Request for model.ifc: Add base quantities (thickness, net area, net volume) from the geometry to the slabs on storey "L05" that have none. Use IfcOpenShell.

First a look at what the model holds.

```python
import ifcopenshell
import ifcopenshell.util.element
import ifcopenshell.util.unit

model = ifcopenshell.open("model.ifc")
print(model.schema)
for unit_type in ("LENGTHUNIT", "AREAUNIT", "VOLUMEUNIT"):
    print(unit_type, ifcopenshell.util.unit.calculate_unit_scale(model, unit_type))
storey = next(s for s in model.by_type("IfcBuildingStorey") if s.Name == "L05")
slabs = [e for e in ifcopenshell.util.element.get_decomposition(storey) if e.is_a("IfcSlab")]
for e in sorted(slabs, key=lambda e: e.id()):
    print(e.id(), e.is_a(), e.Name, list(ifcopenshell.util.element.get_psets(e, qtos_only=True)), sep=" | ")
```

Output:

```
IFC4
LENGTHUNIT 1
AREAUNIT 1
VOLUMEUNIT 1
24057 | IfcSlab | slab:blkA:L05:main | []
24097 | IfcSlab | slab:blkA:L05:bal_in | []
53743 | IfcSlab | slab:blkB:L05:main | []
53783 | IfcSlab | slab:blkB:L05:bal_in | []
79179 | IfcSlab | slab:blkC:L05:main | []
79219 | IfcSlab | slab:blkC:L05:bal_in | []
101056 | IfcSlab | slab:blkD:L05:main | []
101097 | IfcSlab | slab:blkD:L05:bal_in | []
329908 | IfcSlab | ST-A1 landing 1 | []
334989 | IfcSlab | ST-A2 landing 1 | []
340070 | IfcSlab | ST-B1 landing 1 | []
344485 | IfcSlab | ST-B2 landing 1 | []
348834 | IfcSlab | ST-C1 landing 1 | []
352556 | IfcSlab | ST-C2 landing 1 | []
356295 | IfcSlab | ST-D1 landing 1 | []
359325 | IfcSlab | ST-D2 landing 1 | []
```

```python
import ifcopenshell
import ifcopenshell.api.pset
import ifcopenshell.geom
import ifcopenshell.util.element
import ifcopenshell.util.shape
import ifcopenshell.util.unit

model = ifcopenshell.open("model.ifc")
unit_scale = ifcopenshell.util.unit.calculate_unit_scale(model)
area_scale = ifcopenshell.util.unit.calculate_unit_scale(model, "AREAUNIT")
volume_scale = ifcopenshell.util.unit.calculate_unit_scale(model, "VOLUMEUNIT")
settings = ifcopenshell.geom.settings()

storey = next(s for s in model.by_type("IfcBuildingStorey") if s.Name == "L05")
slabs = [e for e in ifcopenshell.util.element.get_decomposition(storey) if e.is_a("IfcSlab")]

for e in sorted(slabs, key=lambda e: e.id()):
    if ifcopenshell.util.element.get_psets(e, qtos_only=True, should_inherit=False):
        continue
    # Geometry comes back in metres, in the element's own axes.
    shape = ifcopenshell.geom.create_shape(settings, e)
    values = {
        "Width": ifcopenshell.util.shape.get_z(shape.geometry) / unit_scale,
        "NetArea": ifcopenshell.util.shape.get_footprint_area(shape.geometry) / area_scale,
        "NetVolume": ifcopenshell.util.shape.get_volume(shape.geometry) / volume_scale,
    }
    qto = ifcopenshell.api.pset.add_qto(model, product=e, name="Qto_SlabBaseQuantities")
    ifcopenshell.api.pset.edit_qto(model, qto=qto, properties=values)
    print(e.id(), {k: round(v, 3) for k, v in values.items()})

model.write("model_rev.ifc")
```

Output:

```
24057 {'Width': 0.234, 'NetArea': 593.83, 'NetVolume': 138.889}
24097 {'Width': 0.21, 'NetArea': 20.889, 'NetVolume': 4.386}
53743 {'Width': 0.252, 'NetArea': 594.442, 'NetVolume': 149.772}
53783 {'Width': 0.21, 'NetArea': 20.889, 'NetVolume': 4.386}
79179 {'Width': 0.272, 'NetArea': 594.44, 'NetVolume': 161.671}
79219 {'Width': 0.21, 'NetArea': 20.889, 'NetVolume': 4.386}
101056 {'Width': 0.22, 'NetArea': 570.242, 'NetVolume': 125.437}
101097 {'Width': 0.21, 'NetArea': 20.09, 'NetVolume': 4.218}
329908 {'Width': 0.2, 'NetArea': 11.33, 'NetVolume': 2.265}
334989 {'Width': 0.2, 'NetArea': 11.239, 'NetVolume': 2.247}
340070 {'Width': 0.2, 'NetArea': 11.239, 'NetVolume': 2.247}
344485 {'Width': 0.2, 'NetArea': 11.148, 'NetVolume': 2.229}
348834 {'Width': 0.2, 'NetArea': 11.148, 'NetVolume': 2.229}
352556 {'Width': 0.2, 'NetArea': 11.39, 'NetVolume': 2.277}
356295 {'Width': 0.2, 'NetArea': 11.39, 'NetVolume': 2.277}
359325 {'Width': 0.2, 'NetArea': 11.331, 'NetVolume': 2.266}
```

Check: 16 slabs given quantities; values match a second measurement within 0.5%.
